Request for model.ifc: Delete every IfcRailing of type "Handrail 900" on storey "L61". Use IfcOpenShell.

First a look at what the model holds.

```python
import ifcopenshell
import ifcopenshell.util.element

model = ifcopenshell.open("model.ifc")
print(model.schema)
storey = next(s for s in model.by_type("IfcBuildingStorey") if s.Name == "L61")
railings = [e for e in ifcopenshell.util.element.get_decomposition(storey) if e.is_a("IfcRailing")]
seen = {}
for e in railings:
    element_type = ifcopenshell.util.element.get_type(e)
    name = element_type.Name if element_type not in (None, e) else None
    seen[name] = seen.get(name, 0) + 1
for name, count in sorted(seen.items(), key=str):
    print(count, "x", name)
```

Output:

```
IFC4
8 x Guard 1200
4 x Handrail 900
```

```python
import ifcopenshell
import ifcopenshell.api.root
import ifcopenshell.util.element

model = ifcopenshell.open("model.ifc")

storey = next(s for s in model.by_type("IfcBuildingStorey") if s.Name == "L61")
railings = [e for e in ifcopenshell.util.element.get_decomposition(storey) if e.is_a("IfcRailing")]
targets = [e for e in railings if (t := ifcopenshell.util.element.get_type(e)) not in (None, e) and t.Name == "Handrail 900"]

for e in targets:
    ifcopenshell.api.root.remove_product(model, product=e)
print(len(targets), "removed")

model.write("model_edited.ifc")
```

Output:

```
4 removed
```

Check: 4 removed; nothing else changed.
